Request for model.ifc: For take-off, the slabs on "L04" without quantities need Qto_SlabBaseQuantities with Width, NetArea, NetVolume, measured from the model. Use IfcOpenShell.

First a look at what the model holds.

```python
import ifcopenshell
import ifcopenshell.util.element
import ifcopenshell.util.unit

model = ifcopenshell.open("model.ifc")
print(model.schema)
for unit_type in ("LENGTHUNIT", "AREAUNIT", "VOLUMEUNIT"):
    print(unit_type, ifcopenshell.util.unit.calculate_unit_scale(model, unit_type))
storey = next(s for s in model.by_type("IfcBuildingStorey") if s.Name == "L04")
slabs = [e for e in ifcopenshell.util.element.get_decomposition(storey) if e.is_a("IfcSlab")]
for e in sorted(slabs, key=lambda e: e.id()):
    print(e.id(), e.is_a(), e.Name, list(ifcopenshell.util.element.get_psets(e, qtos_only=True)), sep=" | ")
```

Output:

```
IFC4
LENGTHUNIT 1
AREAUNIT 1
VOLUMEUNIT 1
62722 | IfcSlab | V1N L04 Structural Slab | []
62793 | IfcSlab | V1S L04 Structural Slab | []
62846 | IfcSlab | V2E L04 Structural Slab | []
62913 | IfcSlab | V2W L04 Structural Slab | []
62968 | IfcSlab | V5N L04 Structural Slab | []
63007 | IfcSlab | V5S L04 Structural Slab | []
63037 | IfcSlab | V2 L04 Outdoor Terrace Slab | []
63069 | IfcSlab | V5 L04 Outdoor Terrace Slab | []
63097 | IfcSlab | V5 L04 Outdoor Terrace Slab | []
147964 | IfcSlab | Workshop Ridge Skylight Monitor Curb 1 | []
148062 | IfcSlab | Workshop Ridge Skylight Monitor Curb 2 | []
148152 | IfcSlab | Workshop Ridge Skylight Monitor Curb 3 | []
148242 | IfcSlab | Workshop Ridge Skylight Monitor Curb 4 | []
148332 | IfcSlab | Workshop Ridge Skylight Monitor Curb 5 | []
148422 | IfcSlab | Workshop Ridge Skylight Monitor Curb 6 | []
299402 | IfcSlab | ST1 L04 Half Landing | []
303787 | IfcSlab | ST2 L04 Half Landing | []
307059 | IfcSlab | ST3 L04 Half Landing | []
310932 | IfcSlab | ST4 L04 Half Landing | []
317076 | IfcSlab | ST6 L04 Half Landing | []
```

```python
import ifcopenshell
import ifcopenshell.api.pset
import ifcopenshell.geom
import ifcopenshell.util.element
import ifcopenshell.util.shape
import ifcopenshell.util.unit

model = ifcopenshell.open("model.ifc")
unit_scale = ifcopenshell.util.unit.calculate_unit_scale(model)
area_scale = ifcopenshell.util.unit.calculate_unit_scale(model, "AREAUNIT")
volume_scale = ifcopenshell.util.unit.calculate_unit_scale(model, "VOLUMEUNIT")
settings = ifcopenshell.geom.settings()

storey = next(s for s in model.by_type("IfcBuildingStorey") if s.Name == "L04")
slabs = [e for e in ifcopenshell.util.element.get_decomposition(storey) if e.is_a("IfcSlab")]

for e in sorted(slabs, key=lambda e: e.id()):
    if ifcopenshell.util.element.get_psets(e, qtos_only=True, should_inherit=False):
        continue
    # Geometry comes back in metres, in the element's own axes.
    shape = ifcopenshell.geom.create_shape(settings, e)
    values = {
        "Width": ifcopenshell.util.shape.get_z(shape.geometry) / unit_scale,
        "NetArea": ifcopenshell.util.shape.get_footprint_area(shape.geometry) / area_scale,
        "NetVolume": ifcopenshell.util.shape.get_volume(shape.geometry) / volume_scale,
    }
    qto = ifcopenshell.api.pset.add_qto(model, product=e, name="Qto_SlabBaseQuantities")
    ifcopenshell.api.pset.edit_qto(model, qto=qto, properties=values)
    print(e.id(), {k: round(v, 3) for k, v in values.items()})

model.write("model_updated.ifc")
```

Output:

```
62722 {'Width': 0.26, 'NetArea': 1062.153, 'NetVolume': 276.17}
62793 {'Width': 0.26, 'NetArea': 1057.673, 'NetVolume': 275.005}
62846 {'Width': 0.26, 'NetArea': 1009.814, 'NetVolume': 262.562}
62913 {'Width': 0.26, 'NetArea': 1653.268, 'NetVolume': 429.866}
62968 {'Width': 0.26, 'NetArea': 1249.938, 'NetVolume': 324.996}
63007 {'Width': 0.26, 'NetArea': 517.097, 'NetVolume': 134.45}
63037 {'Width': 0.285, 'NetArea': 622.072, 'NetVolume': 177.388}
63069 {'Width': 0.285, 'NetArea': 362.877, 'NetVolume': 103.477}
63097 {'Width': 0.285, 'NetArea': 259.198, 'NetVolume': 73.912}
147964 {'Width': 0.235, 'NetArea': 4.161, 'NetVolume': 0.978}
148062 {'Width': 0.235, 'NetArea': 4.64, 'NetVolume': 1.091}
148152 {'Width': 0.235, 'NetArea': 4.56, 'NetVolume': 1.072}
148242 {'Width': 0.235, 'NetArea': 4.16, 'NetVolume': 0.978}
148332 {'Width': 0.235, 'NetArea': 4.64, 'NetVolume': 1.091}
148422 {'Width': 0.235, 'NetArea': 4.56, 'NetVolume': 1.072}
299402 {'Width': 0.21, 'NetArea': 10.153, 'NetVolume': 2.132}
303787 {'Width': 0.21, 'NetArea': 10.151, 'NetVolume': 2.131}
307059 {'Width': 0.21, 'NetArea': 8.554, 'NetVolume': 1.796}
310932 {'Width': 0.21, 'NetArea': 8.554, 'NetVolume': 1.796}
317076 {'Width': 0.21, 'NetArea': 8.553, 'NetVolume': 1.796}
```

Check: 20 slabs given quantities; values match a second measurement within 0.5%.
